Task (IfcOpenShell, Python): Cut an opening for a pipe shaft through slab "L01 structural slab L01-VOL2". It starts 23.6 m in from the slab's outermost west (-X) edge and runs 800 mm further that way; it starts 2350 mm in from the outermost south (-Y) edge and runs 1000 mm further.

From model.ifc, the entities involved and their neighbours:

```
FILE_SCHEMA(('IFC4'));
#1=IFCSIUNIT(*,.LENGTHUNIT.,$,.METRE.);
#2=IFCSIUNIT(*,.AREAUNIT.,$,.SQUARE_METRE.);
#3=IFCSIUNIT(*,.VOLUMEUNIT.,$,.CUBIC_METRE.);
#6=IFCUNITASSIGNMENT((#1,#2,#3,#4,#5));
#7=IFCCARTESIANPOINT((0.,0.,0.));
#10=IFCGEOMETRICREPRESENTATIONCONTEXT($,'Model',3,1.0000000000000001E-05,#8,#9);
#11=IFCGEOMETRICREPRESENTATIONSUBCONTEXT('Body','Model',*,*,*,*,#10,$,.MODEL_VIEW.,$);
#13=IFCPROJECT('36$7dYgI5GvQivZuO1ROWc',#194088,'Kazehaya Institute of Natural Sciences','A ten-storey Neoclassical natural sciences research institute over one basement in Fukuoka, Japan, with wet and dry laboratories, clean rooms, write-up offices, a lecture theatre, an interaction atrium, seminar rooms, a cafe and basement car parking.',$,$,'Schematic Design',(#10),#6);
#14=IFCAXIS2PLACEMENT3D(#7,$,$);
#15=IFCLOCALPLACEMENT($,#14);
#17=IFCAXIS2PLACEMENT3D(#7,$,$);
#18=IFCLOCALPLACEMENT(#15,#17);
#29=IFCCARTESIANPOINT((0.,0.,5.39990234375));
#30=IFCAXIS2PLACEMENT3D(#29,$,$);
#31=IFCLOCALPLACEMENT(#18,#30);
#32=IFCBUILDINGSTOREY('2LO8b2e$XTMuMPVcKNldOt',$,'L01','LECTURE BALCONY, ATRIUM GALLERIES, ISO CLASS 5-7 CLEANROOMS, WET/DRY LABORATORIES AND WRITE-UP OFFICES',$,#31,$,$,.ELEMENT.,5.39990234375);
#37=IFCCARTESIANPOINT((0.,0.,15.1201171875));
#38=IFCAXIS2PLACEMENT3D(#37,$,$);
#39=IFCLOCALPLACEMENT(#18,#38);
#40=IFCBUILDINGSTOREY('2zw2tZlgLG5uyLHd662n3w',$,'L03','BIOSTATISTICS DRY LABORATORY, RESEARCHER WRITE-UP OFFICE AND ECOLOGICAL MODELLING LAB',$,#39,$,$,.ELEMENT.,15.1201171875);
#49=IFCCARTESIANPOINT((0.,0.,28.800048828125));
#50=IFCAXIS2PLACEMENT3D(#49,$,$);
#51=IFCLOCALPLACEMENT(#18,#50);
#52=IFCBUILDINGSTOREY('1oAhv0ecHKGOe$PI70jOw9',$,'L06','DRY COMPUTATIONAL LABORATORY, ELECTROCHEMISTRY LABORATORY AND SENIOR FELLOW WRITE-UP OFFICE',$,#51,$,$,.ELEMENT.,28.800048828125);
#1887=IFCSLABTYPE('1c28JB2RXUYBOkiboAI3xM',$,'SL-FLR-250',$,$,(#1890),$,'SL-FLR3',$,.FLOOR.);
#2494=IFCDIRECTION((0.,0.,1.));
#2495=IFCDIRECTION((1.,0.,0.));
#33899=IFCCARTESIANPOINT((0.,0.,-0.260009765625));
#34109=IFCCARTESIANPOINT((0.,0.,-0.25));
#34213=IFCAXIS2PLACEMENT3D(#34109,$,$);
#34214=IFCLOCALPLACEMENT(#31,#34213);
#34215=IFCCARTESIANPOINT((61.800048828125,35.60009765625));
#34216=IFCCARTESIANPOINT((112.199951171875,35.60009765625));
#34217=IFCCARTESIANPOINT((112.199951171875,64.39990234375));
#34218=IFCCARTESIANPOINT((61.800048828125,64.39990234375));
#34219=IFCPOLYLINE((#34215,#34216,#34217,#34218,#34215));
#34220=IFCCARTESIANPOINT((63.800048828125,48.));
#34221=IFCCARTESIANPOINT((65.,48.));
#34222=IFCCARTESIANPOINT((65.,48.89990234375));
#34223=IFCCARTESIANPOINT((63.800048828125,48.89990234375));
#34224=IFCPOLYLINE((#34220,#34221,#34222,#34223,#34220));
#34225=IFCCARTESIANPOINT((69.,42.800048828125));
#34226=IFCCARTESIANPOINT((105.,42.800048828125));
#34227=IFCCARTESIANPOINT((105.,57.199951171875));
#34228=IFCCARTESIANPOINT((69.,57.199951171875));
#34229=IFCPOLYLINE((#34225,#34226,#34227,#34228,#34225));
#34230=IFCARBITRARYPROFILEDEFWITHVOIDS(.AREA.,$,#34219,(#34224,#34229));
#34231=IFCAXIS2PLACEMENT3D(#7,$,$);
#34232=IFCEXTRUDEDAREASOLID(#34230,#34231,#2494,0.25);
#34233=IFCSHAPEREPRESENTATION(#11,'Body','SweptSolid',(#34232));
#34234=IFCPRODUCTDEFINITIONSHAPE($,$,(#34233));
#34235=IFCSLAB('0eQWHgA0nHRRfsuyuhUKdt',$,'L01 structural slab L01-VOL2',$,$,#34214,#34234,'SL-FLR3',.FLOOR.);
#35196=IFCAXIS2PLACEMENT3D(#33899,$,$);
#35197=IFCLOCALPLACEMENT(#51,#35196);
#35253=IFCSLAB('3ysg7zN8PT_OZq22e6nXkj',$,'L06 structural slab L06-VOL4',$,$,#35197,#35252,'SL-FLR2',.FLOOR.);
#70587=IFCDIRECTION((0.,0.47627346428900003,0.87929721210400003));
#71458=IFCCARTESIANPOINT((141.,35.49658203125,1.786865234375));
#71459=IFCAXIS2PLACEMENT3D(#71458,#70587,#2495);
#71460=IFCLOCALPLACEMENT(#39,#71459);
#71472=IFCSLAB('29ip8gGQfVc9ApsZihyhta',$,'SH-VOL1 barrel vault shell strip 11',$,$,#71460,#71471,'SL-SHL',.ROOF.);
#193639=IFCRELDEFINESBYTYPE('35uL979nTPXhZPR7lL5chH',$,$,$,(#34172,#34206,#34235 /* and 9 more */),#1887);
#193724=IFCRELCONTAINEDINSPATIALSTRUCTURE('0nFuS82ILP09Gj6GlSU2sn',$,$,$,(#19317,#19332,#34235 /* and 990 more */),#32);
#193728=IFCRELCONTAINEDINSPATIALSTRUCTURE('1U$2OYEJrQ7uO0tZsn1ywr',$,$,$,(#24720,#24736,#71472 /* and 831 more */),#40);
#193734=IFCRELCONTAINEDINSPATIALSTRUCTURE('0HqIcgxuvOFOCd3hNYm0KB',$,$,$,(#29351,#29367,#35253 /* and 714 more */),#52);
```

```python
import numpy as np
import ifcopenshell
import ifcopenshell.api.feature
import ifcopenshell.api.geometry
import ifcopenshell.api.root
import ifcopenshell.geom
import ifcopenshell.util.placement
import ifcopenshell.util.representation
import ifcopenshell.util.shape
import ifcopenshell.util.unit

model = ifcopenshell.open("model.ifc")
unit_scale = ifcopenshell.util.unit.calculate_unit_scale(model)
settings = ifcopenshell.geom.settings()


def volume(element):
    """Net volume in cubic metres, openings subtracted."""
    shape = ifcopenshell.geom.create_shape(settings, element)
    return ifcopenshell.util.shape.get_volume(shape.geometry)


slab = model.by_guid("0eQWHgA0nHRRfsuyuhUKdt")
before = volume(slab)

# Extent in the slab's own axes, in metres. The edges named are its -X and -Y sides.
slab_shape = ifcopenshell.geom.create_shape(settings, slab)
vertices = ifcopenshell.util.shape.get_vertices(slab_shape.geometry)
x_min, y_min, bottom = vertices.min(axis=0)
top = vertices[:, 2].max()

opening = ifcopenshell.api.root.create_entity(model, ifc_class="IfcOpeningElement", name="Pipe shaft opening", predefined_type="OPENING")
context = ifcopenshell.util.representation.get_context(model, "Model", "Body", "MODEL_VIEW")
width, depth = 0.8, 1
outline = [(0.0, 0.0), (width, 0.0), (width, depth), (0.0, depth), (0.0, 0.0)]
# Overshoot both faces by 50 mm so the cut is clean.
shape = ifcopenshell.api.geometry.add_slab_representation(
    model, context=context, depth=top - bottom + 0.1, polyline=outline
)
ifcopenshell.api.geometry.assign_representation(model, product=opening, representation=shape)

matrix = ifcopenshell.util.placement.get_local_placement(slab.ObjectPlacement)
matrix[:, 3] = matrix @ np.append(np.array([x_min + 23.6, y_min + 2.35, bottom - 0.05]) / unit_scale, 1.0)
ifcopenshell.api.geometry.edit_object_placement(model, product=opening, matrix=matrix, is_si=False)
ifcopenshell.api.feature.add_feature(model, feature=opening, element=slab)

after = volume(slab)

print(f"slab volume {before:.3f} -> {after:.3f} m3")

model.write("model_rev.ifc")
```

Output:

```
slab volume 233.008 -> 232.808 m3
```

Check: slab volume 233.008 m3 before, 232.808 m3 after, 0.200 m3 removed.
